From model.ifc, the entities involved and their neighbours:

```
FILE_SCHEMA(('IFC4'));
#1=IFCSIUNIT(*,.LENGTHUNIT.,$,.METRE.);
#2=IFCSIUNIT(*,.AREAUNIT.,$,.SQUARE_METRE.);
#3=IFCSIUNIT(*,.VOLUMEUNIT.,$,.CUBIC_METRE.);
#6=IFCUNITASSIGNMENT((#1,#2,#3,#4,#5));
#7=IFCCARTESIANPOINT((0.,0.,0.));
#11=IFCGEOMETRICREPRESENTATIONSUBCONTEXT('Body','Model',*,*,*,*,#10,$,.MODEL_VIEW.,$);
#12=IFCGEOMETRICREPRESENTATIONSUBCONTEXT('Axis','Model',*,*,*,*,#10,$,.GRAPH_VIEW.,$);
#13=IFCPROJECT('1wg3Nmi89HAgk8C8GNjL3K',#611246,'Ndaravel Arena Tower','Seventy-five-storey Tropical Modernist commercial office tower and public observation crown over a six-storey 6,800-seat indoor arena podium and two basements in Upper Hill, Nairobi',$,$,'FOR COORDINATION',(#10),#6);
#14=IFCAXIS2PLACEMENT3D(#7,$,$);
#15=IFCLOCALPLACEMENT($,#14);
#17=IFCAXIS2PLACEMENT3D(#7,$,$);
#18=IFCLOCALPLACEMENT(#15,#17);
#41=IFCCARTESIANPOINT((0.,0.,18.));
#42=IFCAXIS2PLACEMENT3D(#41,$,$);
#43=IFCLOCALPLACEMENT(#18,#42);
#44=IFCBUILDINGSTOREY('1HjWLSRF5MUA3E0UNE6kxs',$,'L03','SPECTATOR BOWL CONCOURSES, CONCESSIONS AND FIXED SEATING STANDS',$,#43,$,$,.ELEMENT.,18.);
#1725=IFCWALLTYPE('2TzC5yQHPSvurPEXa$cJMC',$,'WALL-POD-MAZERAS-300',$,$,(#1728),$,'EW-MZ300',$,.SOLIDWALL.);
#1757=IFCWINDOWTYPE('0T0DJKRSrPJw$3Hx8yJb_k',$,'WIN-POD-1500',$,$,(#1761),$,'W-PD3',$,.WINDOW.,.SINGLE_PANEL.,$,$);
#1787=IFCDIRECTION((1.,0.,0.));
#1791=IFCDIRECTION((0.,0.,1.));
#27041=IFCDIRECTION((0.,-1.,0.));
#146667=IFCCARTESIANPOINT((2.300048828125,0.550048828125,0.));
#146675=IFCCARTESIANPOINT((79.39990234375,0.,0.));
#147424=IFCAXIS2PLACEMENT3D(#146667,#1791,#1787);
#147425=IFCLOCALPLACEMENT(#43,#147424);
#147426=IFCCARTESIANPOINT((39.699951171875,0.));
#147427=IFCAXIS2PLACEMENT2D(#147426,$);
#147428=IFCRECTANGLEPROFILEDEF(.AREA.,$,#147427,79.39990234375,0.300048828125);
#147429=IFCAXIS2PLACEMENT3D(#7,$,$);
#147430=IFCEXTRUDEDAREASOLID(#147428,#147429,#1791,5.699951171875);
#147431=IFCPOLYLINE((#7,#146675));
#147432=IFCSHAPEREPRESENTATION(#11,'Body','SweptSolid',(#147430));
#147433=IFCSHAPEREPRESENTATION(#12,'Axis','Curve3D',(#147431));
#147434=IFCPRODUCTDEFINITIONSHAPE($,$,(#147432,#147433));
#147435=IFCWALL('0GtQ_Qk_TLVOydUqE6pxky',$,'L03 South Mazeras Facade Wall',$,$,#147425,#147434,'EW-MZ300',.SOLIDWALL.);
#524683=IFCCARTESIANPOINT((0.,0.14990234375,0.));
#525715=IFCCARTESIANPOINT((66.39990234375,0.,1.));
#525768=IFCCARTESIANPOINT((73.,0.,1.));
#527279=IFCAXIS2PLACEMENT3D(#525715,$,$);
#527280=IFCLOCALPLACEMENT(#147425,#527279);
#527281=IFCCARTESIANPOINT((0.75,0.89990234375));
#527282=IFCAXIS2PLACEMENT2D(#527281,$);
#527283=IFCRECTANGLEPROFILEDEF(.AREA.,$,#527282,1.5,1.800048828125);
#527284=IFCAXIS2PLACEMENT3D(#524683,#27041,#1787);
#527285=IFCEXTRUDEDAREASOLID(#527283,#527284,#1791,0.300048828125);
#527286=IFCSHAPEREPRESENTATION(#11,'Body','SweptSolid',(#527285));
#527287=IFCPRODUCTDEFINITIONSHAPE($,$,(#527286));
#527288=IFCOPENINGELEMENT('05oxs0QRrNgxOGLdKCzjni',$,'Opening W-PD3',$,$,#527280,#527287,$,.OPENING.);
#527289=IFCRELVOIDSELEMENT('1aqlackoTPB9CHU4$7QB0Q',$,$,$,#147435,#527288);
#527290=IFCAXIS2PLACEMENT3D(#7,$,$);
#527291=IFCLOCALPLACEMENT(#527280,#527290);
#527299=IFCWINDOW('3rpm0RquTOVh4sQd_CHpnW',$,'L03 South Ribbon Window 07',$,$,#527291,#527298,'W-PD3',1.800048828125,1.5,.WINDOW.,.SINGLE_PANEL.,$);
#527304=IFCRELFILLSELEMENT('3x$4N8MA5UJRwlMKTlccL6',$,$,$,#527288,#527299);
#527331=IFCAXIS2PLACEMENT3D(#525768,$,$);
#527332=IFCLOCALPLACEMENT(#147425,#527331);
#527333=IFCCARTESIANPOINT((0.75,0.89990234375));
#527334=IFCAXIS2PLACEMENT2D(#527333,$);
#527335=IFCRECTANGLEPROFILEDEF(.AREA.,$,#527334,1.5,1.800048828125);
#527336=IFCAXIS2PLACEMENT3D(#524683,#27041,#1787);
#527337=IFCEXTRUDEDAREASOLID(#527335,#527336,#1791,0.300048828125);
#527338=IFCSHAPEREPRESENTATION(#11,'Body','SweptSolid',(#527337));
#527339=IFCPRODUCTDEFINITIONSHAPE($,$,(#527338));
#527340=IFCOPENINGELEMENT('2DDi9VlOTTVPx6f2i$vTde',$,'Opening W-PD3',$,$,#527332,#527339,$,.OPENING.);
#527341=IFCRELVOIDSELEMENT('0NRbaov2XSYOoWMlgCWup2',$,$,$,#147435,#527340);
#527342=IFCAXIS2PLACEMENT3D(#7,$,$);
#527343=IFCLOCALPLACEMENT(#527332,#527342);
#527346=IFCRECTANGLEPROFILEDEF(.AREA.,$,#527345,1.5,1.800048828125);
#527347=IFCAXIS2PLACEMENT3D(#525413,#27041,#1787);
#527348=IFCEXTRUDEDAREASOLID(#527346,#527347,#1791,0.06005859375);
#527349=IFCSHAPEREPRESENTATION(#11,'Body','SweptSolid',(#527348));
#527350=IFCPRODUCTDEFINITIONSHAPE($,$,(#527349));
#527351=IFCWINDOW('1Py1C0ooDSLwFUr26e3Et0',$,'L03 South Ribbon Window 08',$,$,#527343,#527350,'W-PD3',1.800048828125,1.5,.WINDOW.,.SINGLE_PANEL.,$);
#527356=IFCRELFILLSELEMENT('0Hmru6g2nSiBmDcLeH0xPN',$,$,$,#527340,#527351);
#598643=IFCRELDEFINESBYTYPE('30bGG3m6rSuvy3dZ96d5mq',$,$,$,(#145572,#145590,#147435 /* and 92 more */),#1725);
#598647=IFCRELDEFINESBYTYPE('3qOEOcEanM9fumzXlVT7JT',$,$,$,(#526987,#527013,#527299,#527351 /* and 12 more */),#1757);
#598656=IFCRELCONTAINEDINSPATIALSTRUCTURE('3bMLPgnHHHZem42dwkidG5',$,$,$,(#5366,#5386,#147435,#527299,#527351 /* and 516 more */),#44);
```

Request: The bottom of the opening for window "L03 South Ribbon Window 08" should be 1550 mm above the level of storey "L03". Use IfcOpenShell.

```python
import numpy as np
import ifcopenshell
import ifcopenshell.api.geometry
import ifcopenshell.geom
import ifcopenshell.util.element
import ifcopenshell.util.placement
import ifcopenshell.util.shape
import ifcopenshell.util.unit

model = ifcopenshell.open("model.ifc")
unit_scale = ifcopenshell.util.unit.calculate_unit_scale(model)

window = model.by_guid("1Py1C0ooDSLwFUr26e3Et0")
opening = window.FillsVoids[0].RelatingOpeningElement
storey = ifcopenshell.util.element.get_container(window, ifc_class="IfcBuildingStorey")
level = ifcopenshell.util.placement.get_local_placement(storey.ObjectPlacement)[2, 3]

# The opening's origin need not be at the sill, so measure its lowest point.
shape = ifcopenshell.geom.create_shape(ifcopenshell.geom.settings(), opening)
bottom = ifcopenshell.util.shape.get_shape_bottom_elevation(shape, shape.geometry) / unit_scale
dz = level + 1.55 - bottom

shift = np.array([0.0, 0.0, dz])
# The window is placed relative to its opening, so it follows when the opening moves.
matrix = ifcopenshell.util.placement.get_local_placement(opening.ObjectPlacement)
matrix[:3, 3] += shift
ifcopenshell.api.geometry.edit_object_placement(
    model, product=opening, matrix=matrix, is_si=False, should_transform_children=True
)

print(f"moved by {dz * unit_scale:+.3f} m")

model.write("model_edited.ifc")
```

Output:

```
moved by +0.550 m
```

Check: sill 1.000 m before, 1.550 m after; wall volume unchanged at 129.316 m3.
